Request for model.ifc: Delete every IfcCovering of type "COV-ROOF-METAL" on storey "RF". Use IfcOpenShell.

First a look at what the model holds.

```python
import ifcopenshell
import ifcopenshell.util.element

model = ifcopenshell.open("model.ifc")
print(model.schema)
storey = next(s for s in model.by_type("IfcBuildingStorey") if s.Name == "RF")
coverings = [e for e in ifcopenshell.util.element.get_decomposition(storey) if e.is_a("IfcCovering")]
seen = {}
for e in coverings:
    element_type = ifcopenshell.util.element.get_type(e)
    name = element_type.Name if element_type not in (None, e) else None
    seen[name] = seen.get(name, 0) + 1
for name, count in sorted(seen.items(), key=str):
    print(count, "x", name)
```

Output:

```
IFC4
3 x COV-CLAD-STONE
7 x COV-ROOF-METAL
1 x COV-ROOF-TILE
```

```python
import ifcopenshell
import ifcopenshell.api.root
import ifcopenshell.util.element

model = ifcopenshell.open("model.ifc")

storey = next(s for s in model.by_type("IfcBuildingStorey") if s.Name == "RF")
coverings = [e for e in ifcopenshell.util.element.get_decomposition(storey) if e.is_a("IfcCovering")]
targets = [e for e in coverings if (t := ifcopenshell.util.element.get_type(e)) not in (None, e) and t.Name == "COV-ROOF-METAL"]

for e in targets:
    ifcopenshell.api.root.remove_product(model, product=e)
print(len(targets), "removed")

model.write("model_updated.ifc")
```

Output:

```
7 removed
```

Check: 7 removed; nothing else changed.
